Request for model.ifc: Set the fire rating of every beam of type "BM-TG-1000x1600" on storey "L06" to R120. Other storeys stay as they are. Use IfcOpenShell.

First a look at what the model holds.

```python
import ifcopenshell
import ifcopenshell.util.element

model = ifcopenshell.open("model.ifc")
print(model.schema)
storey = next(s for s in model.by_type("IfcBuildingStorey") if s.Name == "L06")
beams = [e for e in ifcopenshell.util.element.get_decomposition(storey) if e.is_a("IfcBeam")]
seen = {}
for e in beams:
    element_type = ifcopenshell.util.element.get_type(e)
    key = (element_type.Name if element_type != e and element_type else None, ifcopenshell.util.element.get_pset(e, "Pset_BeamCommon", "FireRating"))
    seen[key] = seen.get(key, 0) + 1
for (name, value), count in sorted(seen.items(), key=str):
    print(count, "x", name, "|", value)
```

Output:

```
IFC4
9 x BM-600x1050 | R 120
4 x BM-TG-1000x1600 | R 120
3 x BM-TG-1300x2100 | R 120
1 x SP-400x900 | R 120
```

```python
import ifcopenshell
import ifcopenshell.api.pset
import ifcopenshell.util.element

model = ifcopenshell.open("model.ifc")

storey = next(s for s in model.by_type("IfcBuildingStorey") if s.Name == "L06")
beams = [e for e in ifcopenshell.util.element.get_decomposition(storey) if e.is_a("IfcBeam")]

count = 0
for e in beams:
    element_type = ifcopenshell.util.element.get_type(e)
    if element_type in (None, e) or element_type.Name != "BM-TG-1000x1600":
        continue
    # add_pset returns the element's existing set when there is one.
    pset = ifcopenshell.api.pset.add_pset(model, product=e, name="Pset_BeamCommon")
    ifcopenshell.api.pset.edit_pset(model, pset=pset, properties={"FireRating": "R120"})
    count += 1

print(count, "beams updated")

model.write("model_updated.ifc")
```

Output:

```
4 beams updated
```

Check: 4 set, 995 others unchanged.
